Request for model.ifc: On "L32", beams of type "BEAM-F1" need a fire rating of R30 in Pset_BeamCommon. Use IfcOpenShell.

First a look at what the model holds.

```python
import ifcopenshell
import ifcopenshell.util.element

model = ifcopenshell.open("model.ifc")
print(model.schema)
storey = next(s for s in model.by_type("IfcBuildingStorey") if s.Name == "L32")
beams = [e for e in ifcopenshell.util.element.get_decomposition(storey) if e.is_a("IfcBeam")]
seen = {}
for e in beams:
    element_type = ifcopenshell.util.element.get_type(e)
    key = (element_type.Name if element_type != e and element_type else None, ifcopenshell.util.element.get_pset(e, "Pset_BeamCommon", "FireRating"))
    seen[key] = seen.get(key, 0) + 1
for (name, value), count in sorted(seen.items(), key=str):
    print(count, "x", name, "|", value)
```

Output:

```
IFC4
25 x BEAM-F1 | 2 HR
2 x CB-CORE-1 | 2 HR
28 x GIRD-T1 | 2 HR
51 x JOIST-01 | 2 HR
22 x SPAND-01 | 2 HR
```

```python
import ifcopenshell
import ifcopenshell.api.pset
import ifcopenshell.util.element

model = ifcopenshell.open("model.ifc")

storey = next(s for s in model.by_type("IfcBuildingStorey") if s.Name == "L32")
beams = [e for e in ifcopenshell.util.element.get_decomposition(storey) if e.is_a("IfcBeam")]

count = 0
for e in beams:
    element_type = ifcopenshell.util.element.get_type(e)
    if element_type in (None, e) or element_type.Name != "BEAM-F1":
        continue
    # add_pset returns the element's existing set when there is one.
    pset = ifcopenshell.api.pset.add_pset(model, product=e, name="Pset_BeamCommon")
    ifcopenshell.api.pset.edit_pset(model, pset=pset, properties={"FireRating": "R30"})
    count += 1

print(count, "beams updated")

model.write("model_rev.ifc")
```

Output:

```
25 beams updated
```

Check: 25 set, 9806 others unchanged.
